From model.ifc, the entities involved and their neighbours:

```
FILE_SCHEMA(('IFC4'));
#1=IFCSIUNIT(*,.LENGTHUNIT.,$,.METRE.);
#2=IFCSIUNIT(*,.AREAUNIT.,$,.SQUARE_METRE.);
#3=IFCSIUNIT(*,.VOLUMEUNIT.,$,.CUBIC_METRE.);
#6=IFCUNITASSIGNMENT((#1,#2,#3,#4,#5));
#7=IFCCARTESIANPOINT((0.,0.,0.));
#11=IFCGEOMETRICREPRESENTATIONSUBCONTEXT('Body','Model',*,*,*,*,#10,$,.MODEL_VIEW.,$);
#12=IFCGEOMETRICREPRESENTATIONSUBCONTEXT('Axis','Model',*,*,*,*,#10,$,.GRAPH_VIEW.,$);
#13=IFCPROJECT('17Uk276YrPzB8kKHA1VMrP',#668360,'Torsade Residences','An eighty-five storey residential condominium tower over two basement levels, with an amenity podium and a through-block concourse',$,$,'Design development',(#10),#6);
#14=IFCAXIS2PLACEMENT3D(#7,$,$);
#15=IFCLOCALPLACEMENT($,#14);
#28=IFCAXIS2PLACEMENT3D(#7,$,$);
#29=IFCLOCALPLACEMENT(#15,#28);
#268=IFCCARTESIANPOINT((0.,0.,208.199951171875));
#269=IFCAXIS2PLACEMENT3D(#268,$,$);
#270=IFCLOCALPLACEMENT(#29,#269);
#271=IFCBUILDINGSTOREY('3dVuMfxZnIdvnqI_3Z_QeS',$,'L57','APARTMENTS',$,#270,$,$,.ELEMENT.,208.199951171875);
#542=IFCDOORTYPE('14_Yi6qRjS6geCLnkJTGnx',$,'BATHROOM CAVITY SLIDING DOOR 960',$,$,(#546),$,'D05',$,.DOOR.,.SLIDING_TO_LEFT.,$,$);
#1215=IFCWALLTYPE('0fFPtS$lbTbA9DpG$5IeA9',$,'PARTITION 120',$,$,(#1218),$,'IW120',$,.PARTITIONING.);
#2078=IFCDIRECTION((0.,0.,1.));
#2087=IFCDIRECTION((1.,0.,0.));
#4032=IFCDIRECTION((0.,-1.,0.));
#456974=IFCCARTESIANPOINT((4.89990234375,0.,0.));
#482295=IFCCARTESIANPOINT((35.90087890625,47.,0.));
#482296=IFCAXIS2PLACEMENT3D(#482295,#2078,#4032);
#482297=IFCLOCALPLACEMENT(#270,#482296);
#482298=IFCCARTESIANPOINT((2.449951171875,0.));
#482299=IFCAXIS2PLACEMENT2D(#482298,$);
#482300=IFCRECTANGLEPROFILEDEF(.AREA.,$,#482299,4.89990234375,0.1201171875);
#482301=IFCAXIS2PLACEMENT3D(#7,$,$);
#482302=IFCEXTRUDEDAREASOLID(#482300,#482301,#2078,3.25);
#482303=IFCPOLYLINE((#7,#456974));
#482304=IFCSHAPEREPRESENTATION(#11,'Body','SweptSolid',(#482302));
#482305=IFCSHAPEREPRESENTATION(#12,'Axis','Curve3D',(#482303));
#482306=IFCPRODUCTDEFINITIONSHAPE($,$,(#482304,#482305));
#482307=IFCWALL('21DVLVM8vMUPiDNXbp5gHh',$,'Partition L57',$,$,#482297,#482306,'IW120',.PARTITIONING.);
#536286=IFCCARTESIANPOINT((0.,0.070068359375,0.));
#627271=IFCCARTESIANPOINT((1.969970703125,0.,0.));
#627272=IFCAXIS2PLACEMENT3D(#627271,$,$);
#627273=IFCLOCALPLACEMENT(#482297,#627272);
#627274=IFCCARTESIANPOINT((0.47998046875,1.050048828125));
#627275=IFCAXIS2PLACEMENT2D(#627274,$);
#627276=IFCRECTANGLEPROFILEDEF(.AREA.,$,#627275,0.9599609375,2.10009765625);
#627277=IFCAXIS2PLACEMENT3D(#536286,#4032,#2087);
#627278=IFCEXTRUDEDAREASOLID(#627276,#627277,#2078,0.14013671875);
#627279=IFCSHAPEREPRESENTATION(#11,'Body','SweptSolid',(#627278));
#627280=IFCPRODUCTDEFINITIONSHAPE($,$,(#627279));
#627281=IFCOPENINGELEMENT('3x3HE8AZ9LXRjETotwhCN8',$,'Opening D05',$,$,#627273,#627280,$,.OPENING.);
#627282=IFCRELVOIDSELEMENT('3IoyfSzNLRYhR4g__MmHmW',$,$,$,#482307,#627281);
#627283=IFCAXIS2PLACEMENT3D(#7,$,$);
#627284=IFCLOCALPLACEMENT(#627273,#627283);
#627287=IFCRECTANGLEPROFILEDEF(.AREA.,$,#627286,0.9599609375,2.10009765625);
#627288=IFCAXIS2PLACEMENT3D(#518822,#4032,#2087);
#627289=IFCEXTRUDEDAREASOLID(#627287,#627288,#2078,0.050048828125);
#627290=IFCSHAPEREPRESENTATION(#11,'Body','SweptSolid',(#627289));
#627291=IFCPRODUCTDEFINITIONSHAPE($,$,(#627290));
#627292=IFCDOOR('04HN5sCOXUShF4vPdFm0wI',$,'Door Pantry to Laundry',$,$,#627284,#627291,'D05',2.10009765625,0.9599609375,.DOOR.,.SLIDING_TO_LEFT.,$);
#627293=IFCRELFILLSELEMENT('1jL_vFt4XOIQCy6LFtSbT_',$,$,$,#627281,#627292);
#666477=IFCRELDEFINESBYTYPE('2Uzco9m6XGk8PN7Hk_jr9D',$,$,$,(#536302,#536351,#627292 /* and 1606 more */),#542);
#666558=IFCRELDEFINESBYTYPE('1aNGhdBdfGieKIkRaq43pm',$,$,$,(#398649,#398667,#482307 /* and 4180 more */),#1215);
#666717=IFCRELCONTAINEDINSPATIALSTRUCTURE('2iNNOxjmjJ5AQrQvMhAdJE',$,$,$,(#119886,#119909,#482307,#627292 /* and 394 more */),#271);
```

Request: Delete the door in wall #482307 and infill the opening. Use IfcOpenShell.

```python
import ifcopenshell
import ifcopenshell.api.feature
import ifcopenshell.api.root
import ifcopenshell.geom
import ifcopenshell.util.shape

model = ifcopenshell.open("model.ifc")
settings = ifcopenshell.geom.settings()


def volume(element):
    """Net volume in cubic metres, openings subtracted."""
    shape = ifcopenshell.geom.create_shape(settings, element)
    return ifcopenshell.util.shape.get_volume(shape.geometry)


door = model.by_guid("04HN5sCOXUShF4vPdFm0wI")
opening = door.FillsVoids[0].RelatingOpeningElement
wall = opening.VoidsElements[0].RelatingBuildingElement
before = volume(wall)

ifcopenshell.api.root.remove_product(model, product=door)
ifcopenshell.api.feature.remove_feature(model, feature=opening)

after = volume(wall)

print(f"wall volume {before:.3f} -> {after:.3f} m3")

model.write("model_rev.ifc")
```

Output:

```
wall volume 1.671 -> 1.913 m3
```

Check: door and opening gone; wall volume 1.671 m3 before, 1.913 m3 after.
